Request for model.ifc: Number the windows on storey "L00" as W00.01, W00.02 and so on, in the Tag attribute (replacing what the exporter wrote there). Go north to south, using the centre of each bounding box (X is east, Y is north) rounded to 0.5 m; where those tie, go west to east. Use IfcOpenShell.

First a look at what the model holds.

```python
import ifcopenshell
import ifcopenshell.util.element
import ifcopenshell.util.placement

model = ifcopenshell.open("model.ifc")
print(model.schema)
storey = next(s for s in model.by_type("IfcBuildingStorey") if s.Name == "L00")
windows = [e for e in ifcopenshell.util.element.get_decomposition(storey) if e.is_a("IfcWindow")]
for e in sorted(windows, key=lambda e: e.id()):
    origin = ifcopenshell.util.placement.get_local_placement(e.ObjectPlacement)[:3, 3]
    print(e.id(), e.Tag, e.Name, origin.round(2) + 0.0, sep=" | ")
```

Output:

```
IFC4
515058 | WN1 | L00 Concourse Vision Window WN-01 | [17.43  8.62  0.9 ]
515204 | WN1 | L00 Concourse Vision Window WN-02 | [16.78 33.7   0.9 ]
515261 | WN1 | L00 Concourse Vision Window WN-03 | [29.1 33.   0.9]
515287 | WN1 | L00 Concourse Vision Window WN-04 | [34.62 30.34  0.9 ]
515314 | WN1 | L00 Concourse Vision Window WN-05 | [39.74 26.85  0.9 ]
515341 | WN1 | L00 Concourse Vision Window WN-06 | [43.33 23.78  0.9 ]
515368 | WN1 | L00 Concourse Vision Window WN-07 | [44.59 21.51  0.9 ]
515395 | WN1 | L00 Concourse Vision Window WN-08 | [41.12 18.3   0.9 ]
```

```python
import ifcopenshell
import ifcopenshell.geom
import ifcopenshell.util.element
import ifcopenshell.util.shape

model = ifcopenshell.open("model.ifc")
settings = ifcopenshell.geom.settings()
settings.set("use-world-coords", True)


def centre(element):
    shape = ifcopenshell.geom.create_shape(settings, element)
    return ifcopenshell.util.shape.get_bbox_centroid(shape.geometry)


storey = next(s for s in model.by_type("IfcBuildingStorey") if s.Name == "L00")
windows = [e for e in ifcopenshell.util.element.get_decomposition(storey) if e.is_a("IfcWindow")]

# Insertion points can sit at a corner or the storey origin, so sort by the geometry (in metres).
centres = {e: centre(e) for e in windows}
windows.sort(key=lambda e: (-round(centres[e][1] / 0.5), centres[e][0]))

for i, e in enumerate(windows, start=1):
    number = f"W00.{i:02d}"
    e.Tag = number
    print(e.id(), number)

model.write("model_updated.ifc")
```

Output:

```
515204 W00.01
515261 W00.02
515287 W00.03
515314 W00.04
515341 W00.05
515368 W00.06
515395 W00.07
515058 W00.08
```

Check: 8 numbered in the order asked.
